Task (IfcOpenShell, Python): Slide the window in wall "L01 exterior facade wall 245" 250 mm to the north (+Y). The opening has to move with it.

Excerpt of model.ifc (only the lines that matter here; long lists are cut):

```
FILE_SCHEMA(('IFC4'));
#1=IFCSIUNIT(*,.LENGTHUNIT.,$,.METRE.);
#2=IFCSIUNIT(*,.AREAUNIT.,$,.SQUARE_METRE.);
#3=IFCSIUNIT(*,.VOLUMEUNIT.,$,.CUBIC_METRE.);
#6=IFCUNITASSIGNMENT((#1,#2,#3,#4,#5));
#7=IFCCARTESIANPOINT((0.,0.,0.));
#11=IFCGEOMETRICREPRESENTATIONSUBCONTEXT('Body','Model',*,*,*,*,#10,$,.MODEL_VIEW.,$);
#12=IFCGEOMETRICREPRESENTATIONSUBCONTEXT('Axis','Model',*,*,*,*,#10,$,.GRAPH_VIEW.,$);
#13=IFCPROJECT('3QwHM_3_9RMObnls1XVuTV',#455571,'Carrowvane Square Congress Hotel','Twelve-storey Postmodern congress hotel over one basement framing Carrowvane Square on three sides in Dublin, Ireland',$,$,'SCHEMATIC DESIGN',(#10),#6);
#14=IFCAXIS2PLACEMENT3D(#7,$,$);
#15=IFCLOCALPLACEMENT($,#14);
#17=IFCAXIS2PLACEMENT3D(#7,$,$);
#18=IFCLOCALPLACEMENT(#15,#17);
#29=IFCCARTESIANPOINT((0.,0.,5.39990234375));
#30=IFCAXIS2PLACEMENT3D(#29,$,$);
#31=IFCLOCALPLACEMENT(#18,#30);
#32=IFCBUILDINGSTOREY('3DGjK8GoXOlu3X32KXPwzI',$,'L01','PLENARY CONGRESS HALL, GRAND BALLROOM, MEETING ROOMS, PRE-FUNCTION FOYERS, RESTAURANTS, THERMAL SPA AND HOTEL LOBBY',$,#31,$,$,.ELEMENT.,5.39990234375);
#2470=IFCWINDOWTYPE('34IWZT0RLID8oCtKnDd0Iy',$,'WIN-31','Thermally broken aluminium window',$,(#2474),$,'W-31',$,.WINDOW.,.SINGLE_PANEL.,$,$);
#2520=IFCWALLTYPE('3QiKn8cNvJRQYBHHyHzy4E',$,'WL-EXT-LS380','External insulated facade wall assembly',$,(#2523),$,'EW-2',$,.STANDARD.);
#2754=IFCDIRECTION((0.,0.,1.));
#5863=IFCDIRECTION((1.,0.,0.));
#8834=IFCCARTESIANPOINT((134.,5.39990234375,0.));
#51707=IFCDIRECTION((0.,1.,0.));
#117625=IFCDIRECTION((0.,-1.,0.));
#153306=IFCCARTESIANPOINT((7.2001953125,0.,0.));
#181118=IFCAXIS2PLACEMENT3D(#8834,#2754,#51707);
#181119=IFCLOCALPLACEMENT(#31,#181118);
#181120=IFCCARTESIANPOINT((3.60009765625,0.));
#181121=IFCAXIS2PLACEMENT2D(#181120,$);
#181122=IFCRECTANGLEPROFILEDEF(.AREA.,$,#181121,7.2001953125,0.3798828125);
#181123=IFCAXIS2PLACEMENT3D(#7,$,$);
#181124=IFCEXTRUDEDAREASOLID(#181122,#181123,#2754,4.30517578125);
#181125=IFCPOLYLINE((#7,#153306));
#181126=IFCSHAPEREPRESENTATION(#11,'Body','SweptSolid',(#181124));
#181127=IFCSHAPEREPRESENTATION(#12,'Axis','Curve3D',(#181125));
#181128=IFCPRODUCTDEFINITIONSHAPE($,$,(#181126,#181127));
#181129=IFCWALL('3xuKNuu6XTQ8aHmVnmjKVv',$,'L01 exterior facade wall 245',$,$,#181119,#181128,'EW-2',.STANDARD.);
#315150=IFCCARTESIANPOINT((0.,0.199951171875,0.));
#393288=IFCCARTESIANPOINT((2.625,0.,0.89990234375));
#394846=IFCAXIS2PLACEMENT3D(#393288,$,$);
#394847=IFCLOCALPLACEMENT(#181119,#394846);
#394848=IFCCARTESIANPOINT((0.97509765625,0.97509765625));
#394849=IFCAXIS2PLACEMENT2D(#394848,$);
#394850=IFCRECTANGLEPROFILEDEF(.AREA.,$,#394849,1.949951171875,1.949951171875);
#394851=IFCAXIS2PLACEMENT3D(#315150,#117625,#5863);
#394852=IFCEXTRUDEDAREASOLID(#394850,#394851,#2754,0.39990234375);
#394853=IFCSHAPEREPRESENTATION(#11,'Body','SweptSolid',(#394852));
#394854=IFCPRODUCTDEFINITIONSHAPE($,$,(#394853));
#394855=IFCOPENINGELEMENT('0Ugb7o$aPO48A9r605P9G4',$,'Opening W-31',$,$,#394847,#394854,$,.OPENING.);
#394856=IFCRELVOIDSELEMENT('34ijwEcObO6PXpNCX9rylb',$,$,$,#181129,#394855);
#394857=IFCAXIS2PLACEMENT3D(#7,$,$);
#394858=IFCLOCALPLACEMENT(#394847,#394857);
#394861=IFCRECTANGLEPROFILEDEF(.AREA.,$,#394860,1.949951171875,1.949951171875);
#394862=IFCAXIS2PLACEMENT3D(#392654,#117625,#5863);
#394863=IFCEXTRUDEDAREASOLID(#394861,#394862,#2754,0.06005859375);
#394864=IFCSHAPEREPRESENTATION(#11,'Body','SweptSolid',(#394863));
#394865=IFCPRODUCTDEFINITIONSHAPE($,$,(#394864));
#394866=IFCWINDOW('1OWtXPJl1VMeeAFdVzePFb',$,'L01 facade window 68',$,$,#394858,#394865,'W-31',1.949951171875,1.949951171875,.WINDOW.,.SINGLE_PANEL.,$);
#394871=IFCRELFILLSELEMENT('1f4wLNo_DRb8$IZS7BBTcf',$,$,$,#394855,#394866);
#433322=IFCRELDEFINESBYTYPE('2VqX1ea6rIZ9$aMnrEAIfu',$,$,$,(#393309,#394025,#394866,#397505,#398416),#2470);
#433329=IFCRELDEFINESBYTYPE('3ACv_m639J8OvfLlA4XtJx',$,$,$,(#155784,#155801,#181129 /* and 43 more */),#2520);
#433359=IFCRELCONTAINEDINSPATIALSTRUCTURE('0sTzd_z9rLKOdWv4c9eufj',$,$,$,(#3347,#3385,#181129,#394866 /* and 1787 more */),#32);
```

```python
import ifcopenshell
import ifcopenshell.api.geometry
import ifcopenshell.util.placement
import ifcopenshell.util.unit

model = ifcopenshell.open("model.ifc")
unit_scale = ifcopenshell.util.unit.calculate_unit_scale(model)

window = model.by_guid("1OWtXPJl1VMeeAFdVzePFb")
opening = window.FillsVoids[0].RelatingOpeningElement
wall = opening.VoidsElements[0].RelatingBuildingElement

wall_matrix = ifcopenshell.util.placement.get_local_placement(wall.ObjectPlacement)
shift = wall_matrix[:3, 0] * 0.25 / unit_scale
before = ifcopenshell.util.placement.get_local_placement(window.ObjectPlacement)[:3, 3].copy()

# The window is placed relative to its opening, so it follows when the opening moves.
matrix = ifcopenshell.util.placement.get_local_placement(opening.ObjectPlacement)
matrix[:3, 3] += shift
ifcopenshell.api.geometry.edit_object_placement(
    model, product=opening, matrix=matrix, is_si=False, should_transform_children=True
)

after = ifcopenshell.util.placement.get_local_placement(window.ObjectPlacement)[:3, 3]
print("window moved by", (after - before).round(3) + 0.0)

model.write("model_updated.ifc")
```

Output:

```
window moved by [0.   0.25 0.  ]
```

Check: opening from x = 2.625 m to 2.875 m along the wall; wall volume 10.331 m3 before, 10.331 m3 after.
